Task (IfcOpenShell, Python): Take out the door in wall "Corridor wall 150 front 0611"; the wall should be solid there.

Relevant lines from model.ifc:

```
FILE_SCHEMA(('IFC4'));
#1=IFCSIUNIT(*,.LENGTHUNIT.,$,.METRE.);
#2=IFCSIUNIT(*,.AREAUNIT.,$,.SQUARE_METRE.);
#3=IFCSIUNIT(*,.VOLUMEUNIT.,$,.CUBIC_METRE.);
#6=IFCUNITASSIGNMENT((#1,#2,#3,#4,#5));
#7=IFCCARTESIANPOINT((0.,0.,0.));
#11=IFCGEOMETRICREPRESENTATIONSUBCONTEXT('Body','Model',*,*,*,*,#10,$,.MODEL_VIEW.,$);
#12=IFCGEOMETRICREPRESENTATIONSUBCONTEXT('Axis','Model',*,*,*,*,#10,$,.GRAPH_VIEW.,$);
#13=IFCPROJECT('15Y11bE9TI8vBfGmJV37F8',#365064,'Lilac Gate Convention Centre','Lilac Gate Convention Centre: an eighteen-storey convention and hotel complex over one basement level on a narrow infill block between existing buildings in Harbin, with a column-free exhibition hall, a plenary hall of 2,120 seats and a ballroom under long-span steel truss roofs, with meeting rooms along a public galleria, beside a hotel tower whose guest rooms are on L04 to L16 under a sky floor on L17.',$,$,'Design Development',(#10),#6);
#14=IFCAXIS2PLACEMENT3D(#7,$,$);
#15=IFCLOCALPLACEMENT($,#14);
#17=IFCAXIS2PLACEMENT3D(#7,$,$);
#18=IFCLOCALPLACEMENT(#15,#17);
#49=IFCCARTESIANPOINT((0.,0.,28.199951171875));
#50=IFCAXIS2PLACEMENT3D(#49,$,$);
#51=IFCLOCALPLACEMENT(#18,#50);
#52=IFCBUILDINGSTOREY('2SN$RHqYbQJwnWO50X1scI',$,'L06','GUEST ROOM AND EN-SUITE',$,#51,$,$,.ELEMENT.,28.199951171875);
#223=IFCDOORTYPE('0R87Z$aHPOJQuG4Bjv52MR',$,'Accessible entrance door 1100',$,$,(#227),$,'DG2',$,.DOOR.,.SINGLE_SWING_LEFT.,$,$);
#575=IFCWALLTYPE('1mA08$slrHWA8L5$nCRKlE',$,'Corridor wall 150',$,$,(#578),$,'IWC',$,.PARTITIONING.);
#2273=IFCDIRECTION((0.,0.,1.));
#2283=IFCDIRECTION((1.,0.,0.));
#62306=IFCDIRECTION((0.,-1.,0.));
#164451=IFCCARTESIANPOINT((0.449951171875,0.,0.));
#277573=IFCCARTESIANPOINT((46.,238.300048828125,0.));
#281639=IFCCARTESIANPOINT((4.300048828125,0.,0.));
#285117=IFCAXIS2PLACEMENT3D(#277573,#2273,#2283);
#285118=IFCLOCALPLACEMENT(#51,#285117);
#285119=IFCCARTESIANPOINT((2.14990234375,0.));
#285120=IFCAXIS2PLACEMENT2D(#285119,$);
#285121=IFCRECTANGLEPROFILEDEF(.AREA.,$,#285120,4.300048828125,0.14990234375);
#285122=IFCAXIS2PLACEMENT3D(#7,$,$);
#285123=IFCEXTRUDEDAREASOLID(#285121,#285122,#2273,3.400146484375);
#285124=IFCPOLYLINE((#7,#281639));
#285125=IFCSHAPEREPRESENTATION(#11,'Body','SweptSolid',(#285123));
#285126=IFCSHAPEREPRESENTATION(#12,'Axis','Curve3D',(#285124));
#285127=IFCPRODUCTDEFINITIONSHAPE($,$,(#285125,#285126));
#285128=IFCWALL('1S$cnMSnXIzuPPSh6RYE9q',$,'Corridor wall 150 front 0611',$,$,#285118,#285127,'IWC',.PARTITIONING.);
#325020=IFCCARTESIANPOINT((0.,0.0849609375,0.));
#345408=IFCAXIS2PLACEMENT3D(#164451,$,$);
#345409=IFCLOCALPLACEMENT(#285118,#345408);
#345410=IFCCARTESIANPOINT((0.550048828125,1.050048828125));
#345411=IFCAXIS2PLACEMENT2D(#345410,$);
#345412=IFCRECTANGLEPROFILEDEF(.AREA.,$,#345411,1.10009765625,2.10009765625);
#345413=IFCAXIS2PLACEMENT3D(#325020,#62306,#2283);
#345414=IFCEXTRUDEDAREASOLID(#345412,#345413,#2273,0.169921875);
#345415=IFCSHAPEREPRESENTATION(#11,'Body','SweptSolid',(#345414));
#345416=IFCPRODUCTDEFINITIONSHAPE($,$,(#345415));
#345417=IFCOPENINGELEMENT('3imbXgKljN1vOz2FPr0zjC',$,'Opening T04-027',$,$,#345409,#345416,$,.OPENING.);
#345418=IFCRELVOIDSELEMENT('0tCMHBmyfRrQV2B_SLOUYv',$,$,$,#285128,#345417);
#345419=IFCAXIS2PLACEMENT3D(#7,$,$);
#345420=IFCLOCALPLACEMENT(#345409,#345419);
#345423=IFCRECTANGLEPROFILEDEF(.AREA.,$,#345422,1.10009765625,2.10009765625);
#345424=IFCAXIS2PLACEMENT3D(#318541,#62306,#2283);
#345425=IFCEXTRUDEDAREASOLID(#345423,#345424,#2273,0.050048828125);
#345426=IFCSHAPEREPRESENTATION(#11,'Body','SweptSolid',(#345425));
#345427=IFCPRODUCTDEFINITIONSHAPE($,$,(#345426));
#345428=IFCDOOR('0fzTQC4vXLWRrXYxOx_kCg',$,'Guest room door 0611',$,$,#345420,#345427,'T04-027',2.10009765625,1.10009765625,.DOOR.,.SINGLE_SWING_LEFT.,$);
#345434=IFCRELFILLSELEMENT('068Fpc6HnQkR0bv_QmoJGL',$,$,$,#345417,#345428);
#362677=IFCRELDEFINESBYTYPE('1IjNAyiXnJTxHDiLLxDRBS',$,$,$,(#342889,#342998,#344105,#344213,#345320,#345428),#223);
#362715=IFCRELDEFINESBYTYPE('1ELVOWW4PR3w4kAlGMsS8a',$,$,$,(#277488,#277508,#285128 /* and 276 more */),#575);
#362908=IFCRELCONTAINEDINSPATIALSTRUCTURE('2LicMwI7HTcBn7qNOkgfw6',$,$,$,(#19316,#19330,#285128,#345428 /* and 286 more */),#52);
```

```python
import ifcopenshell
import ifcopenshell.api.feature
import ifcopenshell.api.root
import ifcopenshell.geom
import ifcopenshell.util.shape

model = ifcopenshell.open("model.ifc")
settings = ifcopenshell.geom.settings()


def volume(element):
    """Net volume in cubic metres, openings subtracted."""
    shape = ifcopenshell.geom.create_shape(settings, element)
    return ifcopenshell.util.shape.get_volume(shape.geometry)


door = model.by_guid("0fzTQC4vXLWRrXYxOx_kCg")
opening = door.FillsVoids[0].RelatingOpeningElement
wall = opening.VoidsElements[0].RelatingBuildingElement
before = volume(wall)

ifcopenshell.api.root.remove_product(model, product=door)
ifcopenshell.api.feature.remove_feature(model, feature=opening)

after = volume(wall)

print(f"wall volume {before:.3f} -> {after:.3f} m3")

model.write("model_updated.ifc")
```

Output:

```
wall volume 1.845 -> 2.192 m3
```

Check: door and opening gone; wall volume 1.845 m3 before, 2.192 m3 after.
